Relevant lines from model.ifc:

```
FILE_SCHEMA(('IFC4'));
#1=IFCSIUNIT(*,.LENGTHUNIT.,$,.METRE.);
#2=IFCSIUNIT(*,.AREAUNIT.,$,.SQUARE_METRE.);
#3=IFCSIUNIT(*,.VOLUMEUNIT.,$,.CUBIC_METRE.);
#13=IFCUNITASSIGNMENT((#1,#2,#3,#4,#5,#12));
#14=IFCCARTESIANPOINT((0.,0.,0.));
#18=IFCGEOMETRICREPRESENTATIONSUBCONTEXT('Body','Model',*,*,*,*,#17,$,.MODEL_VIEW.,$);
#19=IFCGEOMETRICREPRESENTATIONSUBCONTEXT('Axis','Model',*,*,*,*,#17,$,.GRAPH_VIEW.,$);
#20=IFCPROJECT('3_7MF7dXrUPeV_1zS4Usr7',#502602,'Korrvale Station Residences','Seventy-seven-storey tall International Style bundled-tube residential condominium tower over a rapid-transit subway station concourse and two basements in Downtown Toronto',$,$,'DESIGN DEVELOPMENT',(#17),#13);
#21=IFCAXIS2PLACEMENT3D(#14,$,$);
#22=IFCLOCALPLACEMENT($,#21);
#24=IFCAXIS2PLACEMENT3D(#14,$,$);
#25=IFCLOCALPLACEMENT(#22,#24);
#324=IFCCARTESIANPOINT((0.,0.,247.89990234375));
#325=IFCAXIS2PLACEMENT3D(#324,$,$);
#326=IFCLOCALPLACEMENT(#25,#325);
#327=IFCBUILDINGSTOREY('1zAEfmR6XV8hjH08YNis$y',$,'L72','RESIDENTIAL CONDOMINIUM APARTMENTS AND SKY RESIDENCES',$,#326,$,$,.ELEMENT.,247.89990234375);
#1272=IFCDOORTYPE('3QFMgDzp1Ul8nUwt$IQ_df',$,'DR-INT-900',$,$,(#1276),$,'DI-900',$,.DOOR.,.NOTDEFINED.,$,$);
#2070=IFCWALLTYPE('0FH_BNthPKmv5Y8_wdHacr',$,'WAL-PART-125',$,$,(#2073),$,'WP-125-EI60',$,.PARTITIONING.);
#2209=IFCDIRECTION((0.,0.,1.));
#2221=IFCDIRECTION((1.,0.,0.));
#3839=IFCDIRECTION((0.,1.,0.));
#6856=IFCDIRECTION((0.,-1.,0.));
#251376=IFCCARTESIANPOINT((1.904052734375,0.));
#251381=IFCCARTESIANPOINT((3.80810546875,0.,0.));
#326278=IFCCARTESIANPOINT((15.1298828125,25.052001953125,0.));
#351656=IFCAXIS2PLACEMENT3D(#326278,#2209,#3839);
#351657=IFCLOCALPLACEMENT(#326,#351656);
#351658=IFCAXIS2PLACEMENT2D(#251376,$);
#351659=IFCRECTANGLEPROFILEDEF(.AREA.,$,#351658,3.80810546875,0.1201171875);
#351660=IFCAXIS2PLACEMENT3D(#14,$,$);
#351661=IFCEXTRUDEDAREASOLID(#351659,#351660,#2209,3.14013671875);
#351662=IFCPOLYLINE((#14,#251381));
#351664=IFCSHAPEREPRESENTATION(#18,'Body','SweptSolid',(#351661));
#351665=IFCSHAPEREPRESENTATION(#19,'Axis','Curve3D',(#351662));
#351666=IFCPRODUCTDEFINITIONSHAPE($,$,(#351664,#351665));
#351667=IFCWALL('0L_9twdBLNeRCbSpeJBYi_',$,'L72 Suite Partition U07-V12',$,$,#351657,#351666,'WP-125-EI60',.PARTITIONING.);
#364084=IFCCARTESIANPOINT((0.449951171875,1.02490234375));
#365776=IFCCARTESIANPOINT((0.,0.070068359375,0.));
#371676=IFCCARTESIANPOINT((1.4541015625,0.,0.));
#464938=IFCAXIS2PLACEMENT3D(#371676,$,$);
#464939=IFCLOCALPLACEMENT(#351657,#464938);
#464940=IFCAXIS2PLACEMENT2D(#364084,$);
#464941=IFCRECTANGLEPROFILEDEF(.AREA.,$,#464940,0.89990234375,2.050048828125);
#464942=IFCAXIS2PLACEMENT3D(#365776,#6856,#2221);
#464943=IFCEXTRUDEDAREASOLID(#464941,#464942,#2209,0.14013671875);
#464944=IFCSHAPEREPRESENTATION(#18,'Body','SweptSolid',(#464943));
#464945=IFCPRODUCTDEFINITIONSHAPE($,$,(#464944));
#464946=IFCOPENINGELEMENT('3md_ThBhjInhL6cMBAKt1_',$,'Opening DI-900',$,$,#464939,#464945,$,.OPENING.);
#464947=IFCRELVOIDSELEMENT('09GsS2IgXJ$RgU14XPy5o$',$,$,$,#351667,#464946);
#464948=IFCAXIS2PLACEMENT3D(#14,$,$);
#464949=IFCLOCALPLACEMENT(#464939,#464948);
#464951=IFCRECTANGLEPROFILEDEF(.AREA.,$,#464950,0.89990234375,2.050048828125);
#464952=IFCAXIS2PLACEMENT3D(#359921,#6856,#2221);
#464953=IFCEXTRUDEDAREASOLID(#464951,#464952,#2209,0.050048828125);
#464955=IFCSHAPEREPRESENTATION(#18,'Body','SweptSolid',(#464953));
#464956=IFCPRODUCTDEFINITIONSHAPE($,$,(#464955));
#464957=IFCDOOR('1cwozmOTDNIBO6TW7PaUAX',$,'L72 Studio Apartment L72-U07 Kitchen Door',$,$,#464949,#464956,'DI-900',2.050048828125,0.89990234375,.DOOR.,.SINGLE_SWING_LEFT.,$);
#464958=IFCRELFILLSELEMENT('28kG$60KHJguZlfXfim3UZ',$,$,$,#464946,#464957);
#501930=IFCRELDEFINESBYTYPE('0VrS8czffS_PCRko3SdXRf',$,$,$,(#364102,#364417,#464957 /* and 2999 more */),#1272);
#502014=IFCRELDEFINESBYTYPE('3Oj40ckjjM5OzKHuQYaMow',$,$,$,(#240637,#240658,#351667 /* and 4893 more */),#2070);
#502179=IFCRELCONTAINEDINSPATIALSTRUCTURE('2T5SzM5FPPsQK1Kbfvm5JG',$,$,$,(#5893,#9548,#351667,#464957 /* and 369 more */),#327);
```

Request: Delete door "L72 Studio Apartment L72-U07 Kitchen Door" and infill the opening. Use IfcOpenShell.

```python
import ifcopenshell
import ifcopenshell.api.feature
import ifcopenshell.api.root
import ifcopenshell.geom
import ifcopenshell.util.shape

model = ifcopenshell.open("model.ifc")
settings = ifcopenshell.geom.settings()


def volume(element):
    """Net volume in cubic metres, openings subtracted."""
    shape = ifcopenshell.geom.create_shape(settings, element)
    return ifcopenshell.util.shape.get_volume(shape.geometry)


door = model.by_guid("1cwozmOTDNIBO6TW7PaUAX")
opening = door.FillsVoids[0].RelatingOpeningElement
wall = opening.VoidsElements[0].RelatingBuildingElement
before = volume(wall)

ifcopenshell.api.root.remove_product(model, product=door)
ifcopenshell.api.feature.remove_feature(model, feature=opening)

after = volume(wall)

print(f"wall volume {before:.3f} -> {after:.3f} m3")

model.write("model_updated.ifc")
```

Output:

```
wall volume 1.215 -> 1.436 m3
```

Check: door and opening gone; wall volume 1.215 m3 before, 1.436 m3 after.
